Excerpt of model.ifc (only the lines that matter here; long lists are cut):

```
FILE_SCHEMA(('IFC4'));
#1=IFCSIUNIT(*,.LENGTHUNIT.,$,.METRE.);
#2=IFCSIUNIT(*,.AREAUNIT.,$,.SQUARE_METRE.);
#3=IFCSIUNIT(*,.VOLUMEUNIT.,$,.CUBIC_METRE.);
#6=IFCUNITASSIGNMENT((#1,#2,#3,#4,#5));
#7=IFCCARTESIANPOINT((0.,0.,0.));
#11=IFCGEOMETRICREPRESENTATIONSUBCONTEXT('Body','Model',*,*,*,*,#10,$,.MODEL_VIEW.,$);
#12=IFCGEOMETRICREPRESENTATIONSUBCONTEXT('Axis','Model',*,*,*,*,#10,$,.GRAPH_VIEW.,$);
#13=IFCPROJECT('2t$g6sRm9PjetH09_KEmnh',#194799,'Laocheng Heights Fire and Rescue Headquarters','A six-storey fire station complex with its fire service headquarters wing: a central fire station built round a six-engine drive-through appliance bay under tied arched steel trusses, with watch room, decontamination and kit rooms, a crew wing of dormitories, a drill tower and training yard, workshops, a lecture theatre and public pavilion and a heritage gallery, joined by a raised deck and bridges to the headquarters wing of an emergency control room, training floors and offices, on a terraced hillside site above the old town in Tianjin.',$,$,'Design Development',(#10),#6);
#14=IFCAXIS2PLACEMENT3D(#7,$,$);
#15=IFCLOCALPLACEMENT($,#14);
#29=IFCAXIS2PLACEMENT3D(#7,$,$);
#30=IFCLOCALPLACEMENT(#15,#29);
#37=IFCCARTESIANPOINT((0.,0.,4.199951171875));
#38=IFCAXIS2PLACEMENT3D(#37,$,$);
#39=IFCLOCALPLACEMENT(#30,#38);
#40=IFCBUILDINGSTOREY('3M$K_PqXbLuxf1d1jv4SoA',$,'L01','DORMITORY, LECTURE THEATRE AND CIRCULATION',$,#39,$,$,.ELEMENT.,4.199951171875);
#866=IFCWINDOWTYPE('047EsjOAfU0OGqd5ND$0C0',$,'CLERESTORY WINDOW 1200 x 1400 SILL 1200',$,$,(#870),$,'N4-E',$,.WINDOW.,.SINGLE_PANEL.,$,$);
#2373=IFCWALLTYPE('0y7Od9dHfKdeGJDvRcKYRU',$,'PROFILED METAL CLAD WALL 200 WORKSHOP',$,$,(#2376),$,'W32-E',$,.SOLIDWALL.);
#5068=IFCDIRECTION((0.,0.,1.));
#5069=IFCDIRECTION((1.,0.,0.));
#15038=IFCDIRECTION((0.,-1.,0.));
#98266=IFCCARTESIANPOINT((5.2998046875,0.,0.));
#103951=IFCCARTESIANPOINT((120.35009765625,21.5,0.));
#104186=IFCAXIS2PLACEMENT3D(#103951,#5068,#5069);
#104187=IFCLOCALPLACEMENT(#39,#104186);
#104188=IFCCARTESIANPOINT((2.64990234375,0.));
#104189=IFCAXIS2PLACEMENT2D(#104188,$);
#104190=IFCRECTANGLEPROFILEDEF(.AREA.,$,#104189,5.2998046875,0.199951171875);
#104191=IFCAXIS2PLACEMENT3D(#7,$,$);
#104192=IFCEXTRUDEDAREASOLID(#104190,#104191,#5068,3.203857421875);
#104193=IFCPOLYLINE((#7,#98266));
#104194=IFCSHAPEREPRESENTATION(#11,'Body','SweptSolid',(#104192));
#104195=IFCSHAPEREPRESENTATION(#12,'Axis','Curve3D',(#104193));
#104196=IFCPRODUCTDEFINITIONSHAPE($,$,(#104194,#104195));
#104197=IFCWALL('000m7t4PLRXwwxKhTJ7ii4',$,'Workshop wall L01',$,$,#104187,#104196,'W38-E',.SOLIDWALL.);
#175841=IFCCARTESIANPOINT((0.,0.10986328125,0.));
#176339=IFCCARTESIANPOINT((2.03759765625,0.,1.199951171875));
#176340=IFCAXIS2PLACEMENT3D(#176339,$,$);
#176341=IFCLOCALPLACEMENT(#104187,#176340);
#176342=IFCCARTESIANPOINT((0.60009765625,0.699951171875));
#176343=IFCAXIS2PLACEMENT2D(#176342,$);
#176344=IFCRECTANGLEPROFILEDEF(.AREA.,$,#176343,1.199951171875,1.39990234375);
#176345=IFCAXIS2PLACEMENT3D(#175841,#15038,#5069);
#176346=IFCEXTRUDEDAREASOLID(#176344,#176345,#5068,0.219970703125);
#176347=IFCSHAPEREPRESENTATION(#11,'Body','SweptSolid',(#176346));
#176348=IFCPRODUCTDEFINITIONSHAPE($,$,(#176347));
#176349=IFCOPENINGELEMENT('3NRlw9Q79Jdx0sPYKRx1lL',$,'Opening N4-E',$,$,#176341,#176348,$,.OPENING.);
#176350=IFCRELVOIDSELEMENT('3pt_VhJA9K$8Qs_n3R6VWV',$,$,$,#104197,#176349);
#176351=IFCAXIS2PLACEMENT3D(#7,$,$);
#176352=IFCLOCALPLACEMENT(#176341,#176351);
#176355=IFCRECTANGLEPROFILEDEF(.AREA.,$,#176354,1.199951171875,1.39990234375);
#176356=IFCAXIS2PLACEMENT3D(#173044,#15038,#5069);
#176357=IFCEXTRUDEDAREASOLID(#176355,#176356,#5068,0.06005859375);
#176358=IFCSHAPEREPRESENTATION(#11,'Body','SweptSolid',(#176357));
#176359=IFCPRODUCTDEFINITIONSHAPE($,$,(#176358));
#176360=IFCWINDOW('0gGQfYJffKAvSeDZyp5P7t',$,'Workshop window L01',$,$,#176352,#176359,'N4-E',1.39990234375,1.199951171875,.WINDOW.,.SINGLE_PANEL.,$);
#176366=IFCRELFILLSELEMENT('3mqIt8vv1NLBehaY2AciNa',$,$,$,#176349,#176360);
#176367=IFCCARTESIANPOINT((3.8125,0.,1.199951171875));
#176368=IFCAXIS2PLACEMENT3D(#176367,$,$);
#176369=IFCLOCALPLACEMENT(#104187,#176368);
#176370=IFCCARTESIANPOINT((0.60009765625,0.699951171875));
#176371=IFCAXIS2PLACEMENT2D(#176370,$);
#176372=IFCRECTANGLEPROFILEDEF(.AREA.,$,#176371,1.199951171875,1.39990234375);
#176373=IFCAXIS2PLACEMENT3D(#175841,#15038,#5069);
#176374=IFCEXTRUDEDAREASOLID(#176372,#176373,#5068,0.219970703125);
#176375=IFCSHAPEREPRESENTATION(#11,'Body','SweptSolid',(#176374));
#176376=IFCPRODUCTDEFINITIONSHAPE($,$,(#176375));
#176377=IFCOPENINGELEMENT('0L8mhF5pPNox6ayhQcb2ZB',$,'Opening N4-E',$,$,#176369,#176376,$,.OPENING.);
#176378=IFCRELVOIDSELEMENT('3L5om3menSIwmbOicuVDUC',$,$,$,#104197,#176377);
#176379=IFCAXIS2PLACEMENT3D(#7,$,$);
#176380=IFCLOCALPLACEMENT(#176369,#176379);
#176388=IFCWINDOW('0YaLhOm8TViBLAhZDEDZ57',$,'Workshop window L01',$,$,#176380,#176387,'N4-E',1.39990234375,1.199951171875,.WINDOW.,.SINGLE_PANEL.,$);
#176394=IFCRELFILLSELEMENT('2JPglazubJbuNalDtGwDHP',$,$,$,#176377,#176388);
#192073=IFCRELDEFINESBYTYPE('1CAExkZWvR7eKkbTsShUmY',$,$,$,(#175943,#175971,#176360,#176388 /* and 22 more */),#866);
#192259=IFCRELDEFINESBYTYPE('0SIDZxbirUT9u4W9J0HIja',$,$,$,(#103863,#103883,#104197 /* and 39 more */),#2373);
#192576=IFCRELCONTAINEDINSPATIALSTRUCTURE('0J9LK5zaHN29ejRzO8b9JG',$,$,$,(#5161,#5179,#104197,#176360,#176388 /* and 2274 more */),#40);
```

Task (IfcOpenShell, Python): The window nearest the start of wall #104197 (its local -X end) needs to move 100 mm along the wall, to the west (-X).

```python
import ifcopenshell
import ifcopenshell.api.geometry
import ifcopenshell.util.placement

model = ifcopenshell.open("model.ifc")

window = model.by_guid("0gGQfYJffKAvSeDZyp5P7t")
opening = window.FillsVoids[0].RelatingOpeningElement
wall = opening.VoidsElements[0].RelatingBuildingElement

wall_matrix = ifcopenshell.util.placement.get_local_placement(wall.ObjectPlacement)
shift = wall_matrix[:3, 0] * -0.1
before = ifcopenshell.util.placement.get_local_placement(window.ObjectPlacement)[:3, 3].copy()

# The window is placed relative to its opening, so it follows when the opening moves.
matrix = ifcopenshell.util.placement.get_local_placement(opening.ObjectPlacement)
matrix[:3, 3] += shift
ifcopenshell.api.geometry.edit_object_placement(
    model, product=opening, matrix=matrix, is_si=False, should_transform_children=True
)

after = ifcopenshell.util.placement.get_local_placement(window.ObjectPlacement)[:3, 3]
print("window moved by", (after - before).round(3) + 0.0)

model.write("model-out.ifc")
```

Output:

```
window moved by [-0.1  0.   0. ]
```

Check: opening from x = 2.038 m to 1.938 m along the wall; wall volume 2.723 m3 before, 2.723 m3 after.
